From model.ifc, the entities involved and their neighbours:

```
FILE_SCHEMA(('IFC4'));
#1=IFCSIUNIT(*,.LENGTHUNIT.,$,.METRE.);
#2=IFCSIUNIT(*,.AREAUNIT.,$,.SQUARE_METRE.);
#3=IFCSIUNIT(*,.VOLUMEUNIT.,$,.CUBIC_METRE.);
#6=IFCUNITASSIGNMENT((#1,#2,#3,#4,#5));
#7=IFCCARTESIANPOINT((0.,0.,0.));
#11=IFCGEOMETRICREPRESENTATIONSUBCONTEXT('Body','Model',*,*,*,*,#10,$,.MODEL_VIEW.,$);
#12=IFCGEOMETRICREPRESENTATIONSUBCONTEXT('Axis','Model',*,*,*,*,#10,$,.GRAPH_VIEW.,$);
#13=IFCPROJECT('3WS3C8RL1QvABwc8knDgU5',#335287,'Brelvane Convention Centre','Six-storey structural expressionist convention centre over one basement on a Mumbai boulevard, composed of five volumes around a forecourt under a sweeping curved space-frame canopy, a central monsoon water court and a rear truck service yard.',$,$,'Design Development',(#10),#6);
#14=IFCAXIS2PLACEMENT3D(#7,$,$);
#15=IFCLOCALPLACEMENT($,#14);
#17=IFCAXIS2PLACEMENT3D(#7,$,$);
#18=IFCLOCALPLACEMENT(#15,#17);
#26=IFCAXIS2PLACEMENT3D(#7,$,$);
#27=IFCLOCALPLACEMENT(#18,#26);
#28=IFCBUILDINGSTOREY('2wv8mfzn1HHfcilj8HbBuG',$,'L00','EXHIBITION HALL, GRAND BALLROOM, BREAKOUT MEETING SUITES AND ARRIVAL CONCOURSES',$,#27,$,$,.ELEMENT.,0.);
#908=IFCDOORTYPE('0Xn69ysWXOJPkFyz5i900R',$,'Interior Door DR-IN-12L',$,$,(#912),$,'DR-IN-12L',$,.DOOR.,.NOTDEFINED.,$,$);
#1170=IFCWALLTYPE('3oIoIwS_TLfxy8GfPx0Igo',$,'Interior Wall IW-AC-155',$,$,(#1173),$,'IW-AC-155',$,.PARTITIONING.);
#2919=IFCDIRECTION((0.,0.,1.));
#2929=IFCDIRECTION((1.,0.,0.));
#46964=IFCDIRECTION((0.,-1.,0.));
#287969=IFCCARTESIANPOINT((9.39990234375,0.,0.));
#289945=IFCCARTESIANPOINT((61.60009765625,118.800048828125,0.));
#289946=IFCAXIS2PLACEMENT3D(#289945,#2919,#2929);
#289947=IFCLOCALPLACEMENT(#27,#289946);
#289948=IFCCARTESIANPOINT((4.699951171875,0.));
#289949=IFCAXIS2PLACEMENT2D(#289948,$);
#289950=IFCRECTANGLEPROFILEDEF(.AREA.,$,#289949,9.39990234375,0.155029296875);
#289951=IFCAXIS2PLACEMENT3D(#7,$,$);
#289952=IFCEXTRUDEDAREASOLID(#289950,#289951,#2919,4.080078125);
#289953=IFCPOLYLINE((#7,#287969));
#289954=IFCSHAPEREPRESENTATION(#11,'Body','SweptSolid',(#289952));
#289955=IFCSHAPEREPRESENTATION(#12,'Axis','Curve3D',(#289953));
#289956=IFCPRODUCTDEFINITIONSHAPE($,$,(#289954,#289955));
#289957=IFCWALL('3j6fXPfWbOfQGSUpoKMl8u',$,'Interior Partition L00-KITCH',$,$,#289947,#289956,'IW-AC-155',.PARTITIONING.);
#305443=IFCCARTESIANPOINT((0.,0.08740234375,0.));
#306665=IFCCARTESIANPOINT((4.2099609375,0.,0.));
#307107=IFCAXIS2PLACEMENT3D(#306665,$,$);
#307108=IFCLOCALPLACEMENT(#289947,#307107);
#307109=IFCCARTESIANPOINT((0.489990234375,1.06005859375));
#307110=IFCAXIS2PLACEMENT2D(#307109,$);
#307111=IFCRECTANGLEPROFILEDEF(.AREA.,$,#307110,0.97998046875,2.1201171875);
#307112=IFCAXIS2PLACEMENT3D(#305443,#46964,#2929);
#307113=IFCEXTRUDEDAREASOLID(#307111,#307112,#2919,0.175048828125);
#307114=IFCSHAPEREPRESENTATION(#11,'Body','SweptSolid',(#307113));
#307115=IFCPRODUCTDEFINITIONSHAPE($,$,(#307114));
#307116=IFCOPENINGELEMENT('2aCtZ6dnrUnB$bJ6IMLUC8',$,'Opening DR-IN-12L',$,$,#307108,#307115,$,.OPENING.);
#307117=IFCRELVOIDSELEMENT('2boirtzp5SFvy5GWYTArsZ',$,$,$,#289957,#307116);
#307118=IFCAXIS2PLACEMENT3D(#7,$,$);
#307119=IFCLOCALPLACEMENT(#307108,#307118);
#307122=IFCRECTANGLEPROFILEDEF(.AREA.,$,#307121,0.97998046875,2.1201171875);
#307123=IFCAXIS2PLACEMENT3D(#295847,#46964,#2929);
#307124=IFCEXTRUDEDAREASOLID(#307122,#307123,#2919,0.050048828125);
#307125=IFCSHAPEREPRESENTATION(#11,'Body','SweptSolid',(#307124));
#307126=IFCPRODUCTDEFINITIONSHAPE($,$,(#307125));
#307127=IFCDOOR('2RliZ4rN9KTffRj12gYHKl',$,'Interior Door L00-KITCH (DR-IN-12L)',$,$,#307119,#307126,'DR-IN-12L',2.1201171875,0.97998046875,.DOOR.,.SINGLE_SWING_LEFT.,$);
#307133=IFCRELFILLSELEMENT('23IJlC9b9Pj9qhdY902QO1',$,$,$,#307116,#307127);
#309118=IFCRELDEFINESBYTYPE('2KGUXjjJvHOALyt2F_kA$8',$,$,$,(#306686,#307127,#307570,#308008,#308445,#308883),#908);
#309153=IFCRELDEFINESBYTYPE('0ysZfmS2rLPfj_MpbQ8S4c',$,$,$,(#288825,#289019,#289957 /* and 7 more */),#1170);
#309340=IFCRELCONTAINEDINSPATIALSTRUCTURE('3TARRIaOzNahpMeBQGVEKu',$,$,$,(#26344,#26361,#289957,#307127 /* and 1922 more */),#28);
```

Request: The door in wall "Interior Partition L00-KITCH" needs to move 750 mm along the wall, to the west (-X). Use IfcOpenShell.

```python
import ifcopenshell
import ifcopenshell.api.geometry
import ifcopenshell.util.placement

model = ifcopenshell.open("model.ifc")

door = model.by_guid("2RliZ4rN9KTffRj12gYHKl")
opening = door.FillsVoids[0].RelatingOpeningElement
wall = opening.VoidsElements[0].RelatingBuildingElement

wall_matrix = ifcopenshell.util.placement.get_local_placement(wall.ObjectPlacement)
shift = wall_matrix[:3, 0] * -0.75
before = ifcopenshell.util.placement.get_local_placement(door.ObjectPlacement)[:3, 3].copy()

# The door is placed relative to its opening, so it follows when the opening moves.
matrix = ifcopenshell.util.placement.get_local_placement(opening.ObjectPlacement)
matrix[:3, 3] += shift
ifcopenshell.api.geometry.edit_object_placement(
    model, product=opening, matrix=matrix, is_si=False, should_transform_children=True
)

after = ifcopenshell.util.placement.get_local_placement(door.ObjectPlacement)[:3, 3]
print("door moved by", (after - before).round(3) + 0.0)

model.write("model_updated.ifc")
```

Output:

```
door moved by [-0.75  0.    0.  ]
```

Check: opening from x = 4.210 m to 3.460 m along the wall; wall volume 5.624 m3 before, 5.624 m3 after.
